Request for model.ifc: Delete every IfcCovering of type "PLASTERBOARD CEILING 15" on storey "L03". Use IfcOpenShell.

First a look at what the model holds.

```python
import ifcopenshell
import ifcopenshell.util.element

model = ifcopenshell.open("model.ifc")
print(model.schema)
storey = next(s for s in model.by_type("IfcBuildingStorey") if s.Name == "L03")
coverings = [e for e in ifcopenshell.util.element.get_decomposition(storey) if e.is_a("IfcCovering")]
seen = {}
for e in coverings:
    element_type = ifcopenshell.util.element.get_type(e)
    name = element_type.Name if element_type not in (None, e) else None
    seen[name] = seen.get(name, 0) + 1
for name, count in sorted(seen.items(), key=str):
    print(count, "x", name)
```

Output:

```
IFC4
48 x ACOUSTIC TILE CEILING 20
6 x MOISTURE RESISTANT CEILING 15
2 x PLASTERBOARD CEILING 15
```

```python
import ifcopenshell
import ifcopenshell.api.root
import ifcopenshell.util.element

model = ifcopenshell.open("model.ifc")

storey = next(s for s in model.by_type("IfcBuildingStorey") if s.Name == "L03")
coverings = [e for e in ifcopenshell.util.element.get_decomposition(storey) if e.is_a("IfcCovering")]
targets = [e for e in coverings if (t := ifcopenshell.util.element.get_type(e)) not in (None, e) and t.Name == "PLASTERBOARD CEILING 15"]

for e in targets:
    ifcopenshell.api.root.remove_product(model, product=e)
print(len(targets), "removed")

model.write("model_rev.ifc")
```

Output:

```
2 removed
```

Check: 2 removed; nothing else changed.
